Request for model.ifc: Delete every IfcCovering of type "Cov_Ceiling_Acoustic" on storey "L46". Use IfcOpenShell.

First a look at what the model holds.

```python
import ifcopenshell
import ifcopenshell.util.element

model = ifcopenshell.open("model.ifc")
print(model.schema)
storey = next(s for s in model.by_type("IfcBuildingStorey") if s.Name == "L46")
coverings = [e for e in ifcopenshell.util.element.get_decomposition(storey) if e.is_a("IfcCovering")]
seen = {}
for e in coverings:
    element_type = ifcopenshell.util.element.get_type(e)
    name = element_type.Name if element_type not in (None, e) else None
    seen[name] = seen.get(name, 0) + 1
for name, count in sorted(seen.items(), key=str):
    print(count, "x", name)
```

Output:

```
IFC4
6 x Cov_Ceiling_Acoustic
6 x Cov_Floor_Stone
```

```python
import ifcopenshell
import ifcopenshell.api.root
import ifcopenshell.util.element

model = ifcopenshell.open("model.ifc")

storey = next(s for s in model.by_type("IfcBuildingStorey") if s.Name == "L46")
coverings = [e for e in ifcopenshell.util.element.get_decomposition(storey) if e.is_a("IfcCovering")]
targets = [e for e in coverings if (t := ifcopenshell.util.element.get_type(e)) not in (None, e) and t.Name == "Cov_Ceiling_Acoustic"]

for e in targets:
    ifcopenshell.api.root.remove_product(model, product=e)
print(len(targets), "removed")

model.write("model_rev.ifc")
```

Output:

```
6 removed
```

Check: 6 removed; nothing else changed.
